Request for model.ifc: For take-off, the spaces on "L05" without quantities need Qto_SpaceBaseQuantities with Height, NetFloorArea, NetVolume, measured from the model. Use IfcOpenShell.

First a look at what the model holds.

```python
import ifcopenshell
import ifcopenshell.util.element
import ifcopenshell.util.unit

model = ifcopenshell.open("model.ifc")
print(model.schema)
for unit_type in ("LENGTHUNIT", "AREAUNIT", "VOLUMEUNIT"):
    print(unit_type, ifcopenshell.util.unit.calculate_unit_scale(model, unit_type))
storey = next(s for s in model.by_type("IfcBuildingStorey") if s.Name == "L05")
spaces = [e for e in ifcopenshell.util.element.get_decomposition(storey) if e.is_a("IfcSpace")]
for e in sorted(spaces, key=lambda e: e.id()):
    print(e.id(), e.is_a(), e.Name, list(ifcopenshell.util.element.get_psets(e, qtos_only=True)), sep=" | ")
```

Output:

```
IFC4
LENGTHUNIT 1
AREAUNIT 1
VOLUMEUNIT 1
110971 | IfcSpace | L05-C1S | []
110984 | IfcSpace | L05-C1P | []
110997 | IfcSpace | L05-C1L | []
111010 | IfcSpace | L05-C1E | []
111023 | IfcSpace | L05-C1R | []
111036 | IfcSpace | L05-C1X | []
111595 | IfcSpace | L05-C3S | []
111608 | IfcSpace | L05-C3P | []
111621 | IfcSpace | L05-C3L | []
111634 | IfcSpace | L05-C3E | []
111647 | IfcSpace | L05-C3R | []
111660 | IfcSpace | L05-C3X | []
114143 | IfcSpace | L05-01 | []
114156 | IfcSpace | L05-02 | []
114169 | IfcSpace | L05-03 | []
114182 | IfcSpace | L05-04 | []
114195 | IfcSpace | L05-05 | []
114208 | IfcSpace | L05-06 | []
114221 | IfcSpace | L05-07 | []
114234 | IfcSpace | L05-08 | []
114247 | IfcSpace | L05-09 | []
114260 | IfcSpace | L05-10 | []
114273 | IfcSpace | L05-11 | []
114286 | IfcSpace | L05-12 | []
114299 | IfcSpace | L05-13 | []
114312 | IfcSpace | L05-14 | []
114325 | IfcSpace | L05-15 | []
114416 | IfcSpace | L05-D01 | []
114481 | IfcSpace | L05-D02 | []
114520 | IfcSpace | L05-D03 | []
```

```python
import ifcopenshell
import ifcopenshell.api.pset
import ifcopenshell.geom
import ifcopenshell.util.element
import ifcopenshell.util.shape
import ifcopenshell.util.unit

model = ifcopenshell.open("model.ifc")
unit_scale = ifcopenshell.util.unit.calculate_unit_scale(model)
area_scale = ifcopenshell.util.unit.calculate_unit_scale(model, "AREAUNIT")
volume_scale = ifcopenshell.util.unit.calculate_unit_scale(model, "VOLUMEUNIT")
settings = ifcopenshell.geom.settings()

storey = next(s for s in model.by_type("IfcBuildingStorey") if s.Name == "L05")
spaces = [e for e in ifcopenshell.util.element.get_decomposition(storey) if e.is_a("IfcSpace")]

for e in sorted(spaces, key=lambda e: e.id()):
    if ifcopenshell.util.element.get_psets(e, qtos_only=True, should_inherit=False):
        continue
    # Geometry comes back in metres, in the element's own axes.
    shape = ifcopenshell.geom.create_shape(settings, e)
    values = {
        "Height": ifcopenshell.util.shape.get_z(shape.geometry) / unit_scale,
        "NetFloorArea": ifcopenshell.util.shape.get_footprint_area(shape.geometry) / area_scale,
        "NetVolume": ifcopenshell.util.shape.get_volume(shape.geometry) / volume_scale,
    }
    qto = ifcopenshell.api.pset.add_qto(model, product=e, name="Qto_SpaceBaseQuantities")
    ifcopenshell.api.pset.edit_qto(model, qto=qto, properties=values)
    print(e.id(), {k: round(v, 3) for k, v in values.items()})

model.write("model_edited.ifc")
```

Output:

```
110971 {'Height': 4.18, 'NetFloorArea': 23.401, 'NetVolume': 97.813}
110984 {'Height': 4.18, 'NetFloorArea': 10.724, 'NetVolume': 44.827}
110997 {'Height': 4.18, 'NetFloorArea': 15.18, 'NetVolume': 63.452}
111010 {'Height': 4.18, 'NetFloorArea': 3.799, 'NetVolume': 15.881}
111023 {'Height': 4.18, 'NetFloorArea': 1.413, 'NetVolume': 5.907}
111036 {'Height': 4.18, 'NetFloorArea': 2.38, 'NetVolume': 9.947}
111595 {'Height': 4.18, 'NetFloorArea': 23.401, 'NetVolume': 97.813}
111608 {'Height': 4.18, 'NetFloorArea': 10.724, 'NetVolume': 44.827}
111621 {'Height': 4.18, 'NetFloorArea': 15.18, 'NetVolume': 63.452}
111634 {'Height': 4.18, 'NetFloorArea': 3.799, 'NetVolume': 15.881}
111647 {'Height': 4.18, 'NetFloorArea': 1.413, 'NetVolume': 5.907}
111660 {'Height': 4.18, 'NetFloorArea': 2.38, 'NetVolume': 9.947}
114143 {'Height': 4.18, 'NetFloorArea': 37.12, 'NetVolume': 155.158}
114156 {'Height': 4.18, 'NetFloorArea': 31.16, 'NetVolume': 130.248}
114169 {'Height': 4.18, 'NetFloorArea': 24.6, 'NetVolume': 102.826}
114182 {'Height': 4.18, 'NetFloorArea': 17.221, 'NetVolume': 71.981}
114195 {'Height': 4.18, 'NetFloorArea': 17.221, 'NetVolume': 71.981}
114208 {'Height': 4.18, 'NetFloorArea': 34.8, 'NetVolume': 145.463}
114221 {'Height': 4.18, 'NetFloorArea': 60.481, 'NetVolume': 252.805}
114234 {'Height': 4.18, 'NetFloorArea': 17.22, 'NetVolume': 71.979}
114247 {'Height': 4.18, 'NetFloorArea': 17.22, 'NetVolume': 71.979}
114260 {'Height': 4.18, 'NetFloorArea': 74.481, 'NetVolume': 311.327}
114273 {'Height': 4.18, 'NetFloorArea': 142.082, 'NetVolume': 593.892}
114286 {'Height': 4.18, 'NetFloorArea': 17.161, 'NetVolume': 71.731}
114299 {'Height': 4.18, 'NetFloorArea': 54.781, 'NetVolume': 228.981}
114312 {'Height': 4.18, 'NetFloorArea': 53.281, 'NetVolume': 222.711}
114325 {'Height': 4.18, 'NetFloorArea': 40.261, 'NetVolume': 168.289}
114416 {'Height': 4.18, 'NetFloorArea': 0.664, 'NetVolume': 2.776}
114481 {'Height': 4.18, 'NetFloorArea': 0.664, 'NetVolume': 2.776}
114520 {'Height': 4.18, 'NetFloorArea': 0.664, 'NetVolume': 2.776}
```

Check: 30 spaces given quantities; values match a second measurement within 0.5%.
